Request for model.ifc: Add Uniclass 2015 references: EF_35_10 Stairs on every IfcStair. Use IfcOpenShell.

First a look at what the model holds.

```python
import ifcopenshell

model = ifcopenshell.open("model.ifc")
print(model.schema)
print("classifications:", [c.Name for c in model.by_type("IfcClassification")])
for ifc_class in ("IfcDoor", "IfcRoof", "IfcStair", "IfcWall", "IfcWindow"):
    print(ifc_class, len(model.by_type(ifc_class)))
```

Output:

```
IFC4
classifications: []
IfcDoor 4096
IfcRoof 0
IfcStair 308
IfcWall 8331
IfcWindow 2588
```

```python
import ifcopenshell
import ifcopenshell.api.classification

model = ifcopenshell.open("model.ifc")

system = ifcopenshell.api.classification.add_classification(model, classification="Uniclass 2015")

codes = {
    "IfcStair": ("EF_35_10", "Stairs"),
}
for ifc_class, (code, name) in codes.items():
    products = model.by_type(ifc_class)
    ifcopenshell.api.classification.add_reference(
        model, products=products, classification=system, identification=code, name=name
    )
    print(code, len(products))

model.write("model_edited.ifc")
```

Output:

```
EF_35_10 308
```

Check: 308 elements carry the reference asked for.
